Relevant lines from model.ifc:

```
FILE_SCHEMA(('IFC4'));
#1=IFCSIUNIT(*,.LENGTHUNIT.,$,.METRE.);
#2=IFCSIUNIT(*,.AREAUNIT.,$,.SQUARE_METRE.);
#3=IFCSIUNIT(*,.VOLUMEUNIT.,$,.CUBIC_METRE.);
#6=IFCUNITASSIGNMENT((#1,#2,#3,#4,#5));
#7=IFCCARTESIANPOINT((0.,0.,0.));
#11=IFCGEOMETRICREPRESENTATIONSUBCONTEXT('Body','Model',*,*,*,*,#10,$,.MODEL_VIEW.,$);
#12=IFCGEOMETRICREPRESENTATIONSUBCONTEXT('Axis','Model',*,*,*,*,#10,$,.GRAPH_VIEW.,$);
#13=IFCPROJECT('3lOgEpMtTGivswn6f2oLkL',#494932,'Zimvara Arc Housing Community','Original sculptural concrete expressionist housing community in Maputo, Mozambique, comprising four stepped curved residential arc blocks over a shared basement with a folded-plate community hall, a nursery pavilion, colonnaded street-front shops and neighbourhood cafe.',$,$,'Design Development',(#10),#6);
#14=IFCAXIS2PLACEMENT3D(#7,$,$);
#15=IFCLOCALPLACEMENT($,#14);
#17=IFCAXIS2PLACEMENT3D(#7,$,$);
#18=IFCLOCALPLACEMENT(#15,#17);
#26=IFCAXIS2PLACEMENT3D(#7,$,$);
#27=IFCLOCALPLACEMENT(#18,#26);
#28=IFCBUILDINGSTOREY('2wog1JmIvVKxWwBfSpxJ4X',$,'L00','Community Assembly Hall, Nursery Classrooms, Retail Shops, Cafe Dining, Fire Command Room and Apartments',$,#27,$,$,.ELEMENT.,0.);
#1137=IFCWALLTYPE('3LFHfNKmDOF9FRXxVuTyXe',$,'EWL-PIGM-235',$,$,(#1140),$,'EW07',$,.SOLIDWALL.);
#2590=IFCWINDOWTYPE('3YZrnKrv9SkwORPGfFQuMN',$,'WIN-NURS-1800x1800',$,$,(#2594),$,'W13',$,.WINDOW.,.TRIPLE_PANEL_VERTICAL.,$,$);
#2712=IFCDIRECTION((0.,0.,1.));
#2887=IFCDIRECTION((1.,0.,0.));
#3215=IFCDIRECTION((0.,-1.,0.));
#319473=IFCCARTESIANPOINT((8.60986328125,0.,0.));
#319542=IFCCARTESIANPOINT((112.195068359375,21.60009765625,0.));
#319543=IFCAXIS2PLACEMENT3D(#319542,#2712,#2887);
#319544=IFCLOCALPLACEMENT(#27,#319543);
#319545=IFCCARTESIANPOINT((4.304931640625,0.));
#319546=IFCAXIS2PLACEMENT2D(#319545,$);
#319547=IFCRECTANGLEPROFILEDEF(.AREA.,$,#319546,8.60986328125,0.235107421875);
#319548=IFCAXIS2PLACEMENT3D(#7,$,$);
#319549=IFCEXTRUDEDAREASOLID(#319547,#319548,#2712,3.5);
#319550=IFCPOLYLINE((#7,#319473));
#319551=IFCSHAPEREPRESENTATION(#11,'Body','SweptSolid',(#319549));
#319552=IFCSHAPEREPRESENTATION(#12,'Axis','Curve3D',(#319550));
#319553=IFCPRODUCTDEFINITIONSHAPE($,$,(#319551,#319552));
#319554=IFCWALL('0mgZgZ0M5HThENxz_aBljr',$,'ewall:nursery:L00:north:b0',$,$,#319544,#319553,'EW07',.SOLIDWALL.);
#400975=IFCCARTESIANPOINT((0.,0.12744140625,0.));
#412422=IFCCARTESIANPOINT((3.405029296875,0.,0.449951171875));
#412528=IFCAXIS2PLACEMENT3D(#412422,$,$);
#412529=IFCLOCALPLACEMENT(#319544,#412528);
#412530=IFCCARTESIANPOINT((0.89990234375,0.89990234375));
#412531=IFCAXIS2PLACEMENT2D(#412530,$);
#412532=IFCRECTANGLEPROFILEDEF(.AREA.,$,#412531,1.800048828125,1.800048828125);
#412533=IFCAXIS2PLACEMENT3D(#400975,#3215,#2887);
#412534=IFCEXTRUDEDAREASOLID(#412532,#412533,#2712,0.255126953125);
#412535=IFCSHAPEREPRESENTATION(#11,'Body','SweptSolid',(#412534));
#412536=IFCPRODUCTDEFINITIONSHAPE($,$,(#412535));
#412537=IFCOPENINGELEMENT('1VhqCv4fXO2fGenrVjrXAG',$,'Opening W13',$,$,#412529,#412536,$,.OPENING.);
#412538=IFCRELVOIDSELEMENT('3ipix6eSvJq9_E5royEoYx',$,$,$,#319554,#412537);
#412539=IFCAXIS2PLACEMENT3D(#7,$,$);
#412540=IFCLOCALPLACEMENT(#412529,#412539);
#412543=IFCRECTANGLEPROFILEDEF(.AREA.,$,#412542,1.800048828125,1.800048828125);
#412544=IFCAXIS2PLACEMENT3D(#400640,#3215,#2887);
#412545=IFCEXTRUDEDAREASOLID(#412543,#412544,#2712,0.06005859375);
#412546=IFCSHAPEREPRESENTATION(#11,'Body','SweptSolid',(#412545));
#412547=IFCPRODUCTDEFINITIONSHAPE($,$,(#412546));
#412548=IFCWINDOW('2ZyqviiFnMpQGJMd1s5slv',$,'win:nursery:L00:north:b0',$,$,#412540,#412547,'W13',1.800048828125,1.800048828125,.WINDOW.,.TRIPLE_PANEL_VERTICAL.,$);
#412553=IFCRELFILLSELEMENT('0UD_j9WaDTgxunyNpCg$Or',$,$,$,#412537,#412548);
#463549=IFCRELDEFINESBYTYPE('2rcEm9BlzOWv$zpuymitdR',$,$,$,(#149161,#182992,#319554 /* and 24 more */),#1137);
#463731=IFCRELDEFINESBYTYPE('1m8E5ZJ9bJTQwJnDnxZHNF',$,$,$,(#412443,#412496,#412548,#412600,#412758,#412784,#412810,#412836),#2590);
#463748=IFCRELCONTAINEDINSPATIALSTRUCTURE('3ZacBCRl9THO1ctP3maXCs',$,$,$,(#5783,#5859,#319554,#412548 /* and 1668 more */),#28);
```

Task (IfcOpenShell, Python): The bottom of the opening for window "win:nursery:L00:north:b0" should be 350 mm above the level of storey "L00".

```python
import numpy as np
import ifcopenshell
import ifcopenshell.api.geometry
import ifcopenshell.geom
import ifcopenshell.util.element
import ifcopenshell.util.placement
import ifcopenshell.util.shape
import ifcopenshell.util.unit

model = ifcopenshell.open("model.ifc")
unit_scale = ifcopenshell.util.unit.calculate_unit_scale(model)

window = model.by_guid("2ZyqviiFnMpQGJMd1s5slv")
opening = window.FillsVoids[0].RelatingOpeningElement
storey = ifcopenshell.util.element.get_container(window, ifc_class="IfcBuildingStorey")
level = ifcopenshell.util.placement.get_local_placement(storey.ObjectPlacement)[2, 3]

# The opening's origin need not be at the sill, so measure its lowest point.
shape = ifcopenshell.geom.create_shape(ifcopenshell.geom.settings(), opening)
bottom = ifcopenshell.util.shape.get_shape_bottom_elevation(shape, shape.geometry) / unit_scale
dz = level + 0.35 / unit_scale - bottom

shift = np.array([0.0, 0.0, dz])
# The window is placed relative to its opening, so it follows when the opening moves.
matrix = ifcopenshell.util.placement.get_local_placement(opening.ObjectPlacement)
matrix[:3, 3] += shift
ifcopenshell.api.geometry.edit_object_placement(
    model, product=opening, matrix=matrix, is_si=False, should_transform_children=True
)

print(f"moved by {dz * unit_scale:+.3f} m")

model.write("model-out.ifc")
```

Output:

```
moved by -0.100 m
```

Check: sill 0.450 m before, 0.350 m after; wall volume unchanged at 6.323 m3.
